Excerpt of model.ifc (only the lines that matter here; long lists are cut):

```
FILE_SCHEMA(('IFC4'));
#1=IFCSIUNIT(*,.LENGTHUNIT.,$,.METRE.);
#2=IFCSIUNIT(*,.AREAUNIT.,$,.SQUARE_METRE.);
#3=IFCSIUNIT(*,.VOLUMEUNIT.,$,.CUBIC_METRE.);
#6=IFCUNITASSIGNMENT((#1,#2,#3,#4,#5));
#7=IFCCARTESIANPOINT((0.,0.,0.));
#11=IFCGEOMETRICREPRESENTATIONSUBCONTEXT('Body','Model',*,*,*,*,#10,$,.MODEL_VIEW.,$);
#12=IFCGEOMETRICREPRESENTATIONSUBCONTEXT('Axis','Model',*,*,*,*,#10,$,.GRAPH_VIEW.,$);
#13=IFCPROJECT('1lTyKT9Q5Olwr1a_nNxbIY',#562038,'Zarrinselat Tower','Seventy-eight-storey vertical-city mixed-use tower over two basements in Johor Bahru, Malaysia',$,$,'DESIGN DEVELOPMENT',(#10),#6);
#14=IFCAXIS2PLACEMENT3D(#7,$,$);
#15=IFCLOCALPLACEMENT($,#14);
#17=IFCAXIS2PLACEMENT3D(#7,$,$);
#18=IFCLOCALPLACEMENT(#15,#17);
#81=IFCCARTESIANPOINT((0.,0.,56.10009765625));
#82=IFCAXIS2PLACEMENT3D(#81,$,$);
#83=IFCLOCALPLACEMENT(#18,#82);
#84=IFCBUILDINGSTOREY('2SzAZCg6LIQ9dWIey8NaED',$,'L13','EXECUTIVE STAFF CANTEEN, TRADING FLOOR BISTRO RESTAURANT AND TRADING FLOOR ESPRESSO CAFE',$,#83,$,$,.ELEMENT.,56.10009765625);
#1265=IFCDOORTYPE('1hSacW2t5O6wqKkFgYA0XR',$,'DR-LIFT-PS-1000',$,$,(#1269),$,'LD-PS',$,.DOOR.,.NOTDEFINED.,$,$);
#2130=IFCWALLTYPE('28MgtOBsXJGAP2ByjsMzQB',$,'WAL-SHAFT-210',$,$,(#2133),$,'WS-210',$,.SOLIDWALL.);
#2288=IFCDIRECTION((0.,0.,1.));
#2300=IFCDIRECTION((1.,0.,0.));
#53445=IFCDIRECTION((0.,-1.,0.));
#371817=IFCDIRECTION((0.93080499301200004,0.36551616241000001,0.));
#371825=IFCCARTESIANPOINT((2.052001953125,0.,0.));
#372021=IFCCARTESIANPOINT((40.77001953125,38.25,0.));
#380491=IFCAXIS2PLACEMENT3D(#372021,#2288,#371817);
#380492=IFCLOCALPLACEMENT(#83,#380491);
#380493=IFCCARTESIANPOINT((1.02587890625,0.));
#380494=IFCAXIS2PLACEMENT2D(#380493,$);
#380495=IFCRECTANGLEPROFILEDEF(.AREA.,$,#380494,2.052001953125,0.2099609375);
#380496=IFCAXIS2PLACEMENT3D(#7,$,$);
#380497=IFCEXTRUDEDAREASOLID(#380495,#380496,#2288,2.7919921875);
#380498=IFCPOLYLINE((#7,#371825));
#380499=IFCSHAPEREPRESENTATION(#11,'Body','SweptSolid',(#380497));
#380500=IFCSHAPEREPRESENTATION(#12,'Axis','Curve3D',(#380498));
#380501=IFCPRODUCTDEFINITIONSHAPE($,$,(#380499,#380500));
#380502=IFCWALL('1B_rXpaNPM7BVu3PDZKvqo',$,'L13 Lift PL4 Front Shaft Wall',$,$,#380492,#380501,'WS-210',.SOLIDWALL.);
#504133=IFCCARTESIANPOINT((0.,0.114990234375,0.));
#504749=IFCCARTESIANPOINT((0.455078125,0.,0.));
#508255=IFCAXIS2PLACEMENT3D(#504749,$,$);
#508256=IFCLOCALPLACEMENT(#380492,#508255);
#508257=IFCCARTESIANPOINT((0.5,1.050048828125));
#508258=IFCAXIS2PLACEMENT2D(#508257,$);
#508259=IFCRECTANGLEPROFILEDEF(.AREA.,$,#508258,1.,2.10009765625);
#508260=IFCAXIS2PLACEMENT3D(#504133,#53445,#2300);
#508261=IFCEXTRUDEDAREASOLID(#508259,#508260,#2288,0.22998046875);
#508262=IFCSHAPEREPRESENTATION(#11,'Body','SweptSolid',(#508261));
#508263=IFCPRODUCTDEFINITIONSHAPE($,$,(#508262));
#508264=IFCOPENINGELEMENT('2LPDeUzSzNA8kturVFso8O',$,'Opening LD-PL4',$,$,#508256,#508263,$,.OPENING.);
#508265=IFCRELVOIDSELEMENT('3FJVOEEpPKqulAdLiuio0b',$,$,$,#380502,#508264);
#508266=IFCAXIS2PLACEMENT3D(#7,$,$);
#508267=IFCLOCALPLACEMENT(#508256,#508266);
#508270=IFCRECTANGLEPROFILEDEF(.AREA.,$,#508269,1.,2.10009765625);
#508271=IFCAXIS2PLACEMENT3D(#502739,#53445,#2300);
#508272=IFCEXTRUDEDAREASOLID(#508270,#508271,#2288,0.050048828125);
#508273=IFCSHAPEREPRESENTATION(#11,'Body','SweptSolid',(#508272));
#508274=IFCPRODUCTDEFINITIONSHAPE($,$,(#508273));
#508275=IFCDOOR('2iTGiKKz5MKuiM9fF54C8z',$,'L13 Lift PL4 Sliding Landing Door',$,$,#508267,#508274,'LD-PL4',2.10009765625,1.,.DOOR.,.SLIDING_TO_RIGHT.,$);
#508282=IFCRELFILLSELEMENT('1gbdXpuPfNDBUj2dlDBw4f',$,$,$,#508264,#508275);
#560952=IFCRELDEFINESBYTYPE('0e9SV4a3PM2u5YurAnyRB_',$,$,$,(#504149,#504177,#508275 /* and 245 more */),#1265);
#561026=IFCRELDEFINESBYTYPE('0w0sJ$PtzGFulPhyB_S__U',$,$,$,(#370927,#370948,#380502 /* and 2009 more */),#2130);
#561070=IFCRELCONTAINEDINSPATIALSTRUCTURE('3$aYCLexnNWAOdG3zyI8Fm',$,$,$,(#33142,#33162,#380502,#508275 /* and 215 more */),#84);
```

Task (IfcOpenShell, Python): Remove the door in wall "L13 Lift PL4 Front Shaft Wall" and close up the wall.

```python
import ifcopenshell
import ifcopenshell.api.feature
import ifcopenshell.api.root
import ifcopenshell.geom
import ifcopenshell.util.shape

model = ifcopenshell.open("model.ifc")
settings = ifcopenshell.geom.settings()


def volume(element):
    """Net volume in cubic metres, openings subtracted."""
    shape = ifcopenshell.geom.create_shape(settings, element)
    return ifcopenshell.util.shape.get_volume(shape.geometry)


door = model.by_guid("2iTGiKKz5MKuiM9fF54C8z")
opening = door.FillsVoids[0].RelatingOpeningElement
wall = opening.VoidsElements[0].RelatingBuildingElement
before = volume(wall)

ifcopenshell.api.root.remove_product(model, product=door)
ifcopenshell.api.feature.remove_feature(model, feature=opening)

after = volume(wall)

print(f"wall volume {before:.3f} -> {after:.3f} m3")

model.write("model_edited.ifc")
```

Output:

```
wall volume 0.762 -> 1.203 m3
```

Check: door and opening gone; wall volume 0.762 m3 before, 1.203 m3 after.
